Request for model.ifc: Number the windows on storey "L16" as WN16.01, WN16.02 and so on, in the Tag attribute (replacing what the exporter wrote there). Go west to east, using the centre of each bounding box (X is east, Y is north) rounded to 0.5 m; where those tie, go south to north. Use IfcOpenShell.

First a look at what the model holds.

```python
import ifcopenshell
import ifcopenshell.util.element
import ifcopenshell.util.placement

model = ifcopenshell.open("model.ifc")
print(model.schema)
storey = next(s for s in model.by_type("IfcBuildingStorey") if s.Name == "L16")
windows = [e for e in ifcopenshell.util.element.get_decomposition(storey) if e.is_a("IfcWindow")]
for e in sorted(windows, key=lambda e: e.id()):
    origin = ifcopenshell.util.placement.get_local_placement(e.ObjectPlacement)[:3, 3]
    print(e.id(), e.Tag, e.Name, origin.round(2) + 0.0, sep=" | ")
```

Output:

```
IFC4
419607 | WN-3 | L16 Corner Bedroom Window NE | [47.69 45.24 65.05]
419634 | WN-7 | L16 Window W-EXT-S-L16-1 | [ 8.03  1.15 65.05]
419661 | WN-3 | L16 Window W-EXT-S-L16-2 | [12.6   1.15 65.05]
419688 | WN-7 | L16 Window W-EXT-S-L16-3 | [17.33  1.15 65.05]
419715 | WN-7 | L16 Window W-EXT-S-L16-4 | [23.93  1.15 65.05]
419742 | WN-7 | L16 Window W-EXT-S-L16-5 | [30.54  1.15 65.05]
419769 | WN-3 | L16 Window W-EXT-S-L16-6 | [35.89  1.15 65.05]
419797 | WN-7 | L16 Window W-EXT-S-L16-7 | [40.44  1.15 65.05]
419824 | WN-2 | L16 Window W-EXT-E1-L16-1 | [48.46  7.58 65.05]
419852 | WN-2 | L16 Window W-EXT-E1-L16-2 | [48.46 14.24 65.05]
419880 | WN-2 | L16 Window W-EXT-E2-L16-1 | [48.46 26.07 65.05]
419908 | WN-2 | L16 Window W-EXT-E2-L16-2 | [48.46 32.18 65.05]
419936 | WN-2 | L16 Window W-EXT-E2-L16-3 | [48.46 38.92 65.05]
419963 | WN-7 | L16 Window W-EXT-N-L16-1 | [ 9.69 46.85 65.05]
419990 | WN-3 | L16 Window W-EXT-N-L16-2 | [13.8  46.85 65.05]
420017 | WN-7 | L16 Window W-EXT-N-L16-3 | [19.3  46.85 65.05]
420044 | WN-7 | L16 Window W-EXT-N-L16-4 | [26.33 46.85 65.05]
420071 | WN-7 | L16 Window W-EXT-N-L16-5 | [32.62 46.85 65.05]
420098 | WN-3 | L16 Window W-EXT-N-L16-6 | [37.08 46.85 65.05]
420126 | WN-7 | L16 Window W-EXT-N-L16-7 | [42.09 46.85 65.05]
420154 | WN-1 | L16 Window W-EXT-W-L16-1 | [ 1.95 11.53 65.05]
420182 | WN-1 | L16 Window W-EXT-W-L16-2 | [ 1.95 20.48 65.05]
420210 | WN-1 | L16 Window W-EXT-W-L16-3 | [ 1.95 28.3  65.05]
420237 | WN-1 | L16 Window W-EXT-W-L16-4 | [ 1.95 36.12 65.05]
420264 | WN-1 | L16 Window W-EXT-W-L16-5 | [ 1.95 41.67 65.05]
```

```python
import ifcopenshell
import ifcopenshell.geom
import ifcopenshell.util.element
import ifcopenshell.util.shape

model = ifcopenshell.open("model.ifc")
settings = ifcopenshell.geom.settings()
settings.set("use-world-coords", True)


def centre(element):
    shape = ifcopenshell.geom.create_shape(settings, element)
    return ifcopenshell.util.shape.get_bbox_centroid(shape.geometry)


storey = next(s for s in model.by_type("IfcBuildingStorey") if s.Name == "L16")
windows = [e for e in ifcopenshell.util.element.get_decomposition(storey) if e.is_a("IfcWindow")]

# Insertion points can sit at a corner or the storey origin, so sort by the geometry (in metres).
centres = {e: centre(e) for e in windows}
windows.sort(key=lambda e: (round(centres[e][0] / 0.5), centres[e][1]))

for i, e in enumerate(windows, start=1):
    number = f"WN16.{i:02d}"
    e.Tag = number
    print(e.id(), number)

model.write("model_edited.ifc")
```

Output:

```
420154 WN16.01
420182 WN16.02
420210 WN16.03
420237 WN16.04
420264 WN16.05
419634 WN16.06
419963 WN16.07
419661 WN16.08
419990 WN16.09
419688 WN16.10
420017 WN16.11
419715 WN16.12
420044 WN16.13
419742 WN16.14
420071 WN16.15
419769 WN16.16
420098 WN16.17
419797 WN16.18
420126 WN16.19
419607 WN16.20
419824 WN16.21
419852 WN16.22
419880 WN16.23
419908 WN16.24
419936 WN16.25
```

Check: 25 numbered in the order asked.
